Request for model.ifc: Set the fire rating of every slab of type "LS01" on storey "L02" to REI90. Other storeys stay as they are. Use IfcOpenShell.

First a look at what the model holds.

```python
import ifcopenshell
import ifcopenshell.util.element

model = ifcopenshell.open("model.ifc")
print(model.schema)
storey = next(s for s in model.by_type("IfcBuildingStorey") if s.Name == "L02")
slabs = [e for e in ifcopenshell.util.element.get_decomposition(storey) if e.is_a("IfcSlab")]
seen = {}
for e in slabs:
    element_type = ifcopenshell.util.element.get_type(e)
    key = (element_type.Name if element_type != e and element_type else None, ifcopenshell.util.element.get_pset(e, "Pset_SlabCommon", "FireRating"))
    seen[key] = seen.get(key, 0) + 1
for (name, value), count in sorted(seen.items(), key=str):
    print(count, "x", name, "|", value)
```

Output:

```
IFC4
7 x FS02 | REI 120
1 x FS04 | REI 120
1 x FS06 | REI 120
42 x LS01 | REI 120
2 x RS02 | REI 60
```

```python
import ifcopenshell
import ifcopenshell.api.pset
import ifcopenshell.util.element

model = ifcopenshell.open("model.ifc")

storey = next(s for s in model.by_type("IfcBuildingStorey") if s.Name == "L02")
slabs = [e for e in ifcopenshell.util.element.get_decomposition(storey) if e.is_a("IfcSlab")]

count = 0
for e in slabs:
    element_type = ifcopenshell.util.element.get_type(e)
    if element_type in (None, e) or element_type.Name != "LS01":
        continue
    # add_pset returns the element's existing set when there is one.
    pset = ifcopenshell.api.pset.add_pset(model, product=e, name="Pset_SlabCommon")
    ifcopenshell.api.pset.edit_pset(model, pset=pset, properties={"FireRating": "REI90"})
    count += 1

print(count, "slabs updated")

model.write("model-out.ifc")
```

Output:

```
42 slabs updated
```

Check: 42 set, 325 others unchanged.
